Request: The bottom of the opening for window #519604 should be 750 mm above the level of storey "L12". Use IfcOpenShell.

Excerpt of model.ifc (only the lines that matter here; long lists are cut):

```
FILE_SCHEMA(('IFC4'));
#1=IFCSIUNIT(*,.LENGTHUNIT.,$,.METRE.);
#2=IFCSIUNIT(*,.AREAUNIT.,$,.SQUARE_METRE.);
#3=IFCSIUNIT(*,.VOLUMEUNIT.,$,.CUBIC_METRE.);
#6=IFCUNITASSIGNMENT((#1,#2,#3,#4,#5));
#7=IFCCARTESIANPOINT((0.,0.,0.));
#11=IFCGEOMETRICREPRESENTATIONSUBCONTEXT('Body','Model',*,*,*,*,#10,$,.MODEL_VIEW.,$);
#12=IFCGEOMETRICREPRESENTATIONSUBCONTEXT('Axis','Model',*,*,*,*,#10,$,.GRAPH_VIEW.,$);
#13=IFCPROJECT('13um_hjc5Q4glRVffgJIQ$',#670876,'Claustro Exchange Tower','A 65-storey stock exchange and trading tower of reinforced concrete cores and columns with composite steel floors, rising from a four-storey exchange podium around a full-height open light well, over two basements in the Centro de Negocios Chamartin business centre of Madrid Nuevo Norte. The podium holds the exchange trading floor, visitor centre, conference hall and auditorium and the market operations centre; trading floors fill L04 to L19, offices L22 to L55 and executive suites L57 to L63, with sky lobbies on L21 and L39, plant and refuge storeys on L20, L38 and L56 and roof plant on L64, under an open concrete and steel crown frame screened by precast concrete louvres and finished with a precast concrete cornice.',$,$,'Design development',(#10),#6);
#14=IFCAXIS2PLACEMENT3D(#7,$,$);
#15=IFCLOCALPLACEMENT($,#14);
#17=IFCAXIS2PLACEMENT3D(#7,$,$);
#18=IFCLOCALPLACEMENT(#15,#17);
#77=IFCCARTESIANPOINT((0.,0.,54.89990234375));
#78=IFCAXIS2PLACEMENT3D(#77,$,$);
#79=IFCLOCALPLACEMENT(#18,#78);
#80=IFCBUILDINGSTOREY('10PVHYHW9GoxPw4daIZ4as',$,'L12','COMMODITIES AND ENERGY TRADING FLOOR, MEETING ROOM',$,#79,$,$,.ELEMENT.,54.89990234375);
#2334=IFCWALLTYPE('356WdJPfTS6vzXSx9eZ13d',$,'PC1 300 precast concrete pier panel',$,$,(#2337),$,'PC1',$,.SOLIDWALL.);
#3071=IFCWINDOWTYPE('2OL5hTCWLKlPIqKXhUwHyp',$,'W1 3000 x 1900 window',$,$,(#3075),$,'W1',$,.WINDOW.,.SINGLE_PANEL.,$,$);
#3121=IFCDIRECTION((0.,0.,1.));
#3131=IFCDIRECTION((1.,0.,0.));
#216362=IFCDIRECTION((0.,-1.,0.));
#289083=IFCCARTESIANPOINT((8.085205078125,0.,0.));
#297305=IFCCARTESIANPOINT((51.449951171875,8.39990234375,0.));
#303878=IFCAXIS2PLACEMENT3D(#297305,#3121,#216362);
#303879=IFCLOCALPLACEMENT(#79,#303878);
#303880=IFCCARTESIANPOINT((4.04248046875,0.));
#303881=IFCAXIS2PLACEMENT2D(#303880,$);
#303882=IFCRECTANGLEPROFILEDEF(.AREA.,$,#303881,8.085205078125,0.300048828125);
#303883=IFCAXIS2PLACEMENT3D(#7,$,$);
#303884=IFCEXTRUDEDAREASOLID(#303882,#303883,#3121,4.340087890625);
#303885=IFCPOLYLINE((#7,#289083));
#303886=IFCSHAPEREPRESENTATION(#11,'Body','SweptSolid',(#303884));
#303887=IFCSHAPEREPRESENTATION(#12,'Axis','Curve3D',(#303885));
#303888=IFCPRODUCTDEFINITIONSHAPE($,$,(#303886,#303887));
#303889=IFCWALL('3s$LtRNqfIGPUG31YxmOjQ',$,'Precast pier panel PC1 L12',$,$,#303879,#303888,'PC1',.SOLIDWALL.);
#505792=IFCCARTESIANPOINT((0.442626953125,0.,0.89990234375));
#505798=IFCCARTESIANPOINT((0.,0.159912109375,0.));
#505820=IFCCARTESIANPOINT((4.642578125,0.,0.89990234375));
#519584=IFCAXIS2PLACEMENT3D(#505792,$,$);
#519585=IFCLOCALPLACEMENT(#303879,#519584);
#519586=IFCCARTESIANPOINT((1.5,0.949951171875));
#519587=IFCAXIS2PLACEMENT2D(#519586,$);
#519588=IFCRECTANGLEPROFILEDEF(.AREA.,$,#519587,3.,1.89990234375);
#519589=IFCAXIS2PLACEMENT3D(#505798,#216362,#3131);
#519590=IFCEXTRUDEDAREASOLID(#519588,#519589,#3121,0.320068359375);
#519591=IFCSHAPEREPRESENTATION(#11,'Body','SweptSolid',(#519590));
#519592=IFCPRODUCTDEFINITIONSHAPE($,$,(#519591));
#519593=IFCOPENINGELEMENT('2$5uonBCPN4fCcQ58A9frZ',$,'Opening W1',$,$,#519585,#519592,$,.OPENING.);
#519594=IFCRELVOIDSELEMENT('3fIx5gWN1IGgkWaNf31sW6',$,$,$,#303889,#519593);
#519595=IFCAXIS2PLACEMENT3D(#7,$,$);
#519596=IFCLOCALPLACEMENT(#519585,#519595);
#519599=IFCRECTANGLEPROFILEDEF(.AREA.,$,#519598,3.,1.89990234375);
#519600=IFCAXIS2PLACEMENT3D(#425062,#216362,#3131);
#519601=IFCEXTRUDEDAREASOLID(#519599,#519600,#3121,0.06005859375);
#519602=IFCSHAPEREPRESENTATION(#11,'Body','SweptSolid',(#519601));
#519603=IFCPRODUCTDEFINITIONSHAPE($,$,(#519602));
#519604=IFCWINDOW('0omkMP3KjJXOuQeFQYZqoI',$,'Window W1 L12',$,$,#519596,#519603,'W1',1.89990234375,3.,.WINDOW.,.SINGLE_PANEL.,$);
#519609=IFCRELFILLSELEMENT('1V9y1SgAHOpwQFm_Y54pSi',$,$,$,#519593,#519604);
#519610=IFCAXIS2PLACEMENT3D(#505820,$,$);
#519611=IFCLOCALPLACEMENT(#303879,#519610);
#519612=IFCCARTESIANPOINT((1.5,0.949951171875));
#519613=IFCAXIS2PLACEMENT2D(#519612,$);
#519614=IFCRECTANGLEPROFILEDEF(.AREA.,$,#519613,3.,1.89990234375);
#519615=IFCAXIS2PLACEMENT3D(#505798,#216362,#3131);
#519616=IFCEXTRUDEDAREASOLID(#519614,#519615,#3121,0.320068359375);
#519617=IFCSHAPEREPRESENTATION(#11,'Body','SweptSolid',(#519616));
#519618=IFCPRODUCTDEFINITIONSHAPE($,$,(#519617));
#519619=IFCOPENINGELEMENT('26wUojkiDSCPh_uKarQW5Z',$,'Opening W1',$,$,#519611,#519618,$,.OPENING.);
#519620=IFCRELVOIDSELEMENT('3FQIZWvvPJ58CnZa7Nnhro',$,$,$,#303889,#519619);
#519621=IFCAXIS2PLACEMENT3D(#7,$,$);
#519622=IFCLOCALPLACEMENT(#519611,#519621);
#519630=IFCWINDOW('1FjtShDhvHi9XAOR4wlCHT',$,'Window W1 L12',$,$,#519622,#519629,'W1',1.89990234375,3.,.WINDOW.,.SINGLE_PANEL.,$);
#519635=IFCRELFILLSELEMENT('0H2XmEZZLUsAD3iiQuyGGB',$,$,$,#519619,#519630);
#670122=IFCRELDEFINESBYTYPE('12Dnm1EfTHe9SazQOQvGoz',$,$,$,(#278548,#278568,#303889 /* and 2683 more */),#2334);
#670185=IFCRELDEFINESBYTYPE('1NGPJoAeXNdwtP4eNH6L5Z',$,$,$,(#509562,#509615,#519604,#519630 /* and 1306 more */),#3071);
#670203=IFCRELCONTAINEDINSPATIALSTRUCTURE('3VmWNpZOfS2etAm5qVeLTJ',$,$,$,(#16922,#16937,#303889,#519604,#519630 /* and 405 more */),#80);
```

```python
import numpy as np
import ifcopenshell
import ifcopenshell.api.geometry
import ifcopenshell.geom
import ifcopenshell.util.element
import ifcopenshell.util.placement
import ifcopenshell.util.shape
import ifcopenshell.util.unit

model = ifcopenshell.open("model.ifc")
unit_scale = ifcopenshell.util.unit.calculate_unit_scale(model)

window = model.by_guid("0omkMP3KjJXOuQeFQYZqoI")
opening = window.FillsVoids[0].RelatingOpeningElement
storey = ifcopenshell.util.element.get_container(window, ifc_class="IfcBuildingStorey")
level = ifcopenshell.util.placement.get_local_placement(storey.ObjectPlacement)[2, 3]

# The opening's origin need not be at the sill, so measure its lowest point.
shape = ifcopenshell.geom.create_shape(ifcopenshell.geom.settings(), opening)
bottom = ifcopenshell.util.shape.get_shape_bottom_elevation(shape, shape.geometry) / unit_scale
dz = level + 0.75 / unit_scale - bottom

shift = np.array([0.0, 0.0, dz])
# The window is placed relative to its opening, so it follows when the opening moves.
matrix = ifcopenshell.util.placement.get_local_placement(opening.ObjectPlacement)
matrix[:3, 3] += shift
ifcopenshell.api.geometry.edit_object_placement(
    model, product=opening, matrix=matrix, is_si=False, should_transform_children=True
)

print(f"moved by {dz * unit_scale:+.3f} m")

model.write("model_rev.ifc")
```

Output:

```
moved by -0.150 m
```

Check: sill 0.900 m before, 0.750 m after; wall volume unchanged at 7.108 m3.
